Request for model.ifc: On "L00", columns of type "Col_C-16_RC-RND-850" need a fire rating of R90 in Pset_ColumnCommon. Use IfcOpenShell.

First a look at what the model holds.

```python
import ifcopenshell
import ifcopenshell.util.element

model = ifcopenshell.open("model.ifc")
print(model.schema)
storey = next(s for s in model.by_type("IfcBuildingStorey") if s.Name == "L00")
columns = [e for e in ifcopenshell.util.element.get_decomposition(storey) if e.is_a("IfcColumn")]
seen = {}
for e in columns:
    element_type = ifcopenshell.util.element.get_type(e)
    key = (element_type.Name if element_type != e and element_type else None, ifcopenshell.util.element.get_pset(e, "Pset_ColumnCommon", "FireRating"))
    seen[key] = seen.get(key, 0) + 1
for (name, value), count in sorted(seen.items(), key=str):
    print(count, "x", name, "|", value)
```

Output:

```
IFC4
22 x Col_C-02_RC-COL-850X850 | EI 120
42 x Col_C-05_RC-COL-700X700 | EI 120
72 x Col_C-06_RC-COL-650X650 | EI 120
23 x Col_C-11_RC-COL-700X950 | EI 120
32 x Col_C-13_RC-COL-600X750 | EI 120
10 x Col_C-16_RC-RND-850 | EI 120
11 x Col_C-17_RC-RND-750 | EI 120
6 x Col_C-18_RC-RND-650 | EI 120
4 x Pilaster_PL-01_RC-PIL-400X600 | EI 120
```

```python
import ifcopenshell
import ifcopenshell.api.pset
import ifcopenshell.util.element

model = ifcopenshell.open("model.ifc")

storey = next(s for s in model.by_type("IfcBuildingStorey") if s.Name == "L00")
columns = [e for e in ifcopenshell.util.element.get_decomposition(storey) if e.is_a("IfcColumn")]

count = 0
for e in columns:
    element_type = ifcopenshell.util.element.get_type(e)
    if element_type in (None, e) or element_type.Name != "Col_C-16_RC-RND-850":
        continue
    # add_pset returns the element's existing set when there is one.
    pset = ifcopenshell.api.pset.add_pset(model, product=e, name="Pset_ColumnCommon")
    ifcopenshell.api.pset.edit_pset(model, pset=pset, properties={"FireRating": "R90"})
    count += 1

print(count, "columns updated")

model.write("model_rev.ifc")
```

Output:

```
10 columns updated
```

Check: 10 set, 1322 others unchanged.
